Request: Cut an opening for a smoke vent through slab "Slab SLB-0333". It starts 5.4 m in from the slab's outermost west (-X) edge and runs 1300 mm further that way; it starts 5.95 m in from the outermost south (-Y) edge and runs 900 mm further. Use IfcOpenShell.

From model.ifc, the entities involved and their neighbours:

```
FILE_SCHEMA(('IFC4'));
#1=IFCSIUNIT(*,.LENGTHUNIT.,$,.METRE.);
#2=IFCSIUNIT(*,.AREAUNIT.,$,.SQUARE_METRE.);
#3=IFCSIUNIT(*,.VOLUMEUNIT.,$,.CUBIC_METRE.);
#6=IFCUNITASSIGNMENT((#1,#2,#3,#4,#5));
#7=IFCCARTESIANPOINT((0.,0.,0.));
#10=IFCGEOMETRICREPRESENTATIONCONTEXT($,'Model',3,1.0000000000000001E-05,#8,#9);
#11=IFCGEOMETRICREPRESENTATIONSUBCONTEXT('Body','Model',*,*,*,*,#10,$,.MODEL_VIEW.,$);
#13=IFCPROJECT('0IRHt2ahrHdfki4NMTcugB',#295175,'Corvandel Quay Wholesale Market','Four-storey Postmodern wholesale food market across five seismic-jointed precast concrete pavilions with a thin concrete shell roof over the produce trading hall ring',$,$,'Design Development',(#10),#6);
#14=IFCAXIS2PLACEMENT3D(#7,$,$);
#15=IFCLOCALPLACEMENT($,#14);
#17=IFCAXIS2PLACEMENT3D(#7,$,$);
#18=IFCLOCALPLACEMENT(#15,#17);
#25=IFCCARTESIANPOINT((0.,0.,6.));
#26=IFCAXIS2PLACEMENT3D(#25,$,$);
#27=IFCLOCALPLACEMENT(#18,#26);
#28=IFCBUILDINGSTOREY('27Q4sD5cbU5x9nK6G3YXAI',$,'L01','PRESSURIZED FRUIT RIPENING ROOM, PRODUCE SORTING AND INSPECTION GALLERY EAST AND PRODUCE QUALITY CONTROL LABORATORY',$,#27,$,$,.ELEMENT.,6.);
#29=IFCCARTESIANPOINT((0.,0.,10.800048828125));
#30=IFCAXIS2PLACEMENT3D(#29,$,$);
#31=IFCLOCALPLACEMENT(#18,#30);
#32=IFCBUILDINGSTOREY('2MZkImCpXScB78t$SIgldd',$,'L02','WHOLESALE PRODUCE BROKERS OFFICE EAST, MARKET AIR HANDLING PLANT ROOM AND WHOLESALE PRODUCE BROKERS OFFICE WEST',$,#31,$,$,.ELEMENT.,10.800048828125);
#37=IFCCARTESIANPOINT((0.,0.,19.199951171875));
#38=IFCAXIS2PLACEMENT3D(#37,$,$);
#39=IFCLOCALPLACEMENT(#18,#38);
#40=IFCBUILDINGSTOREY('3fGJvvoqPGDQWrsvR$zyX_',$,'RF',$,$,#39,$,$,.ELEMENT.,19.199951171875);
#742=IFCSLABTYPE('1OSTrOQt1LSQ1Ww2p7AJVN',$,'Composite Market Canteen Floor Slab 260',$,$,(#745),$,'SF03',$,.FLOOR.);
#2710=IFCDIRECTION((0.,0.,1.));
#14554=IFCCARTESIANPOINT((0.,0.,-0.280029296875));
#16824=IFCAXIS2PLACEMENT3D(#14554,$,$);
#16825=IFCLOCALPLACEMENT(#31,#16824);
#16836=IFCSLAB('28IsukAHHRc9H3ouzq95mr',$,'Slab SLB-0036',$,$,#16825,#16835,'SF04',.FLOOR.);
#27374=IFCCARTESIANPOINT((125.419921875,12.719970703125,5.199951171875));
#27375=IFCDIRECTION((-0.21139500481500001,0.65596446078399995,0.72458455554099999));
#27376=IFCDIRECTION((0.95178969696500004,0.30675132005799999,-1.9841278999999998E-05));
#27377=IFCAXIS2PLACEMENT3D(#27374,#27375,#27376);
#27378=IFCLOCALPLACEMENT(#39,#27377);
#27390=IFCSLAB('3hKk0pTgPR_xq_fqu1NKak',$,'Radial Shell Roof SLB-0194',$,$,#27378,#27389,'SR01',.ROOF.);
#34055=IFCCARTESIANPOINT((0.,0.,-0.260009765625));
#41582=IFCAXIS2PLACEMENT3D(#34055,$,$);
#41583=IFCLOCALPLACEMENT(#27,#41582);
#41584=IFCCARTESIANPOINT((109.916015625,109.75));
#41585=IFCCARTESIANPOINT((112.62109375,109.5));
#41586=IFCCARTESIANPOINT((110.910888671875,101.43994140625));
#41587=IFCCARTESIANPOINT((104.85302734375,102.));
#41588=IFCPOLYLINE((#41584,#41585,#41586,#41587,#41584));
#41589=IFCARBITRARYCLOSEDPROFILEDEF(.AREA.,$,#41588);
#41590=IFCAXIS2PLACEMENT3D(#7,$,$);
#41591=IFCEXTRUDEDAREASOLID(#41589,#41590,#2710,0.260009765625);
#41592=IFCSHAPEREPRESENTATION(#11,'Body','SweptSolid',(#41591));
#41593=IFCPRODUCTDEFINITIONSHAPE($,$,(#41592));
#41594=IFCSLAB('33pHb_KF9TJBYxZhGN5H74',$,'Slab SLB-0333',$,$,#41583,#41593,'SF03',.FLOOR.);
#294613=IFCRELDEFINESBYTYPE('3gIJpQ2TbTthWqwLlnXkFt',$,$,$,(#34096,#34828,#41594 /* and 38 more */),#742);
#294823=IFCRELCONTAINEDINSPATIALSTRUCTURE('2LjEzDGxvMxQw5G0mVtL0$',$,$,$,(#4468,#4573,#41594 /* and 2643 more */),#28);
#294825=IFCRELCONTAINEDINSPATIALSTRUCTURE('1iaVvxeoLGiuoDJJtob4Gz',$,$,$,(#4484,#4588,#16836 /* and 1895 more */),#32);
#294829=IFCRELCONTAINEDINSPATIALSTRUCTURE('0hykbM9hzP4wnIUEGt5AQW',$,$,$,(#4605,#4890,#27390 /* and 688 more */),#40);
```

```python
import numpy as np
import ifcopenshell
import ifcopenshell.api.feature
import ifcopenshell.api.geometry
import ifcopenshell.api.root
import ifcopenshell.geom
import ifcopenshell.util.placement
import ifcopenshell.util.representation
import ifcopenshell.util.shape
import ifcopenshell.util.unit

model = ifcopenshell.open("model.ifc")
unit_scale = ifcopenshell.util.unit.calculate_unit_scale(model)
settings = ifcopenshell.geom.settings()


def volume(element):
    """Net volume in cubic metres, openings subtracted."""
    shape = ifcopenshell.geom.create_shape(settings, element)
    return ifcopenshell.util.shape.get_volume(shape.geometry)


slab = model.by_id(41594)
before = volume(slab)

# Extent in the slab's own axes, in metres. The edges named are its -X and -Y sides.
slab_shape = ifcopenshell.geom.create_shape(settings, slab)
vertices = ifcopenshell.util.shape.get_vertices(slab_shape.geometry)
x_min, y_min, bottom = vertices.min(axis=0)
top = vertices[:, 2].max()

opening = ifcopenshell.api.root.create_entity(model, ifc_class="IfcOpeningElement", name="Smoke vent opening", predefined_type="OPENING")
context = ifcopenshell.util.representation.get_context(model, "Model", "Body", "MODEL_VIEW")
width, depth = 1.3, 0.9
outline = [(0.0, 0.0), (width, 0.0), (width, depth), (0.0, depth), (0.0, 0.0)]
# Overshoot both faces by 50 mm so the cut is clean.
shape = ifcopenshell.api.geometry.add_slab_representation(
    model, context=context, depth=top - bottom + 0.1, polyline=outline
)
ifcopenshell.api.geometry.assign_representation(model, product=opening, representation=shape)

matrix = ifcopenshell.util.placement.get_local_placement(slab.ObjectPlacement)
matrix[:, 3] = matrix @ np.append(np.array([x_min + 5.4, y_min + 5.95, bottom - 0.05]) / unit_scale, 1.0)
ifcopenshell.api.geometry.edit_object_placement(model, product=opening, matrix=matrix, is_si=False)
ifcopenshell.api.feature.add_feature(model, feature=opening, element=slab)

after = volume(slab)

print(f"slab volume {before:.3f} -> {after:.3f} m3")

model.write("model_rev.ifc")
```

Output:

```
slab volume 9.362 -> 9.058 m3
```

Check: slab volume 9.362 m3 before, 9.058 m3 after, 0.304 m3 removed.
